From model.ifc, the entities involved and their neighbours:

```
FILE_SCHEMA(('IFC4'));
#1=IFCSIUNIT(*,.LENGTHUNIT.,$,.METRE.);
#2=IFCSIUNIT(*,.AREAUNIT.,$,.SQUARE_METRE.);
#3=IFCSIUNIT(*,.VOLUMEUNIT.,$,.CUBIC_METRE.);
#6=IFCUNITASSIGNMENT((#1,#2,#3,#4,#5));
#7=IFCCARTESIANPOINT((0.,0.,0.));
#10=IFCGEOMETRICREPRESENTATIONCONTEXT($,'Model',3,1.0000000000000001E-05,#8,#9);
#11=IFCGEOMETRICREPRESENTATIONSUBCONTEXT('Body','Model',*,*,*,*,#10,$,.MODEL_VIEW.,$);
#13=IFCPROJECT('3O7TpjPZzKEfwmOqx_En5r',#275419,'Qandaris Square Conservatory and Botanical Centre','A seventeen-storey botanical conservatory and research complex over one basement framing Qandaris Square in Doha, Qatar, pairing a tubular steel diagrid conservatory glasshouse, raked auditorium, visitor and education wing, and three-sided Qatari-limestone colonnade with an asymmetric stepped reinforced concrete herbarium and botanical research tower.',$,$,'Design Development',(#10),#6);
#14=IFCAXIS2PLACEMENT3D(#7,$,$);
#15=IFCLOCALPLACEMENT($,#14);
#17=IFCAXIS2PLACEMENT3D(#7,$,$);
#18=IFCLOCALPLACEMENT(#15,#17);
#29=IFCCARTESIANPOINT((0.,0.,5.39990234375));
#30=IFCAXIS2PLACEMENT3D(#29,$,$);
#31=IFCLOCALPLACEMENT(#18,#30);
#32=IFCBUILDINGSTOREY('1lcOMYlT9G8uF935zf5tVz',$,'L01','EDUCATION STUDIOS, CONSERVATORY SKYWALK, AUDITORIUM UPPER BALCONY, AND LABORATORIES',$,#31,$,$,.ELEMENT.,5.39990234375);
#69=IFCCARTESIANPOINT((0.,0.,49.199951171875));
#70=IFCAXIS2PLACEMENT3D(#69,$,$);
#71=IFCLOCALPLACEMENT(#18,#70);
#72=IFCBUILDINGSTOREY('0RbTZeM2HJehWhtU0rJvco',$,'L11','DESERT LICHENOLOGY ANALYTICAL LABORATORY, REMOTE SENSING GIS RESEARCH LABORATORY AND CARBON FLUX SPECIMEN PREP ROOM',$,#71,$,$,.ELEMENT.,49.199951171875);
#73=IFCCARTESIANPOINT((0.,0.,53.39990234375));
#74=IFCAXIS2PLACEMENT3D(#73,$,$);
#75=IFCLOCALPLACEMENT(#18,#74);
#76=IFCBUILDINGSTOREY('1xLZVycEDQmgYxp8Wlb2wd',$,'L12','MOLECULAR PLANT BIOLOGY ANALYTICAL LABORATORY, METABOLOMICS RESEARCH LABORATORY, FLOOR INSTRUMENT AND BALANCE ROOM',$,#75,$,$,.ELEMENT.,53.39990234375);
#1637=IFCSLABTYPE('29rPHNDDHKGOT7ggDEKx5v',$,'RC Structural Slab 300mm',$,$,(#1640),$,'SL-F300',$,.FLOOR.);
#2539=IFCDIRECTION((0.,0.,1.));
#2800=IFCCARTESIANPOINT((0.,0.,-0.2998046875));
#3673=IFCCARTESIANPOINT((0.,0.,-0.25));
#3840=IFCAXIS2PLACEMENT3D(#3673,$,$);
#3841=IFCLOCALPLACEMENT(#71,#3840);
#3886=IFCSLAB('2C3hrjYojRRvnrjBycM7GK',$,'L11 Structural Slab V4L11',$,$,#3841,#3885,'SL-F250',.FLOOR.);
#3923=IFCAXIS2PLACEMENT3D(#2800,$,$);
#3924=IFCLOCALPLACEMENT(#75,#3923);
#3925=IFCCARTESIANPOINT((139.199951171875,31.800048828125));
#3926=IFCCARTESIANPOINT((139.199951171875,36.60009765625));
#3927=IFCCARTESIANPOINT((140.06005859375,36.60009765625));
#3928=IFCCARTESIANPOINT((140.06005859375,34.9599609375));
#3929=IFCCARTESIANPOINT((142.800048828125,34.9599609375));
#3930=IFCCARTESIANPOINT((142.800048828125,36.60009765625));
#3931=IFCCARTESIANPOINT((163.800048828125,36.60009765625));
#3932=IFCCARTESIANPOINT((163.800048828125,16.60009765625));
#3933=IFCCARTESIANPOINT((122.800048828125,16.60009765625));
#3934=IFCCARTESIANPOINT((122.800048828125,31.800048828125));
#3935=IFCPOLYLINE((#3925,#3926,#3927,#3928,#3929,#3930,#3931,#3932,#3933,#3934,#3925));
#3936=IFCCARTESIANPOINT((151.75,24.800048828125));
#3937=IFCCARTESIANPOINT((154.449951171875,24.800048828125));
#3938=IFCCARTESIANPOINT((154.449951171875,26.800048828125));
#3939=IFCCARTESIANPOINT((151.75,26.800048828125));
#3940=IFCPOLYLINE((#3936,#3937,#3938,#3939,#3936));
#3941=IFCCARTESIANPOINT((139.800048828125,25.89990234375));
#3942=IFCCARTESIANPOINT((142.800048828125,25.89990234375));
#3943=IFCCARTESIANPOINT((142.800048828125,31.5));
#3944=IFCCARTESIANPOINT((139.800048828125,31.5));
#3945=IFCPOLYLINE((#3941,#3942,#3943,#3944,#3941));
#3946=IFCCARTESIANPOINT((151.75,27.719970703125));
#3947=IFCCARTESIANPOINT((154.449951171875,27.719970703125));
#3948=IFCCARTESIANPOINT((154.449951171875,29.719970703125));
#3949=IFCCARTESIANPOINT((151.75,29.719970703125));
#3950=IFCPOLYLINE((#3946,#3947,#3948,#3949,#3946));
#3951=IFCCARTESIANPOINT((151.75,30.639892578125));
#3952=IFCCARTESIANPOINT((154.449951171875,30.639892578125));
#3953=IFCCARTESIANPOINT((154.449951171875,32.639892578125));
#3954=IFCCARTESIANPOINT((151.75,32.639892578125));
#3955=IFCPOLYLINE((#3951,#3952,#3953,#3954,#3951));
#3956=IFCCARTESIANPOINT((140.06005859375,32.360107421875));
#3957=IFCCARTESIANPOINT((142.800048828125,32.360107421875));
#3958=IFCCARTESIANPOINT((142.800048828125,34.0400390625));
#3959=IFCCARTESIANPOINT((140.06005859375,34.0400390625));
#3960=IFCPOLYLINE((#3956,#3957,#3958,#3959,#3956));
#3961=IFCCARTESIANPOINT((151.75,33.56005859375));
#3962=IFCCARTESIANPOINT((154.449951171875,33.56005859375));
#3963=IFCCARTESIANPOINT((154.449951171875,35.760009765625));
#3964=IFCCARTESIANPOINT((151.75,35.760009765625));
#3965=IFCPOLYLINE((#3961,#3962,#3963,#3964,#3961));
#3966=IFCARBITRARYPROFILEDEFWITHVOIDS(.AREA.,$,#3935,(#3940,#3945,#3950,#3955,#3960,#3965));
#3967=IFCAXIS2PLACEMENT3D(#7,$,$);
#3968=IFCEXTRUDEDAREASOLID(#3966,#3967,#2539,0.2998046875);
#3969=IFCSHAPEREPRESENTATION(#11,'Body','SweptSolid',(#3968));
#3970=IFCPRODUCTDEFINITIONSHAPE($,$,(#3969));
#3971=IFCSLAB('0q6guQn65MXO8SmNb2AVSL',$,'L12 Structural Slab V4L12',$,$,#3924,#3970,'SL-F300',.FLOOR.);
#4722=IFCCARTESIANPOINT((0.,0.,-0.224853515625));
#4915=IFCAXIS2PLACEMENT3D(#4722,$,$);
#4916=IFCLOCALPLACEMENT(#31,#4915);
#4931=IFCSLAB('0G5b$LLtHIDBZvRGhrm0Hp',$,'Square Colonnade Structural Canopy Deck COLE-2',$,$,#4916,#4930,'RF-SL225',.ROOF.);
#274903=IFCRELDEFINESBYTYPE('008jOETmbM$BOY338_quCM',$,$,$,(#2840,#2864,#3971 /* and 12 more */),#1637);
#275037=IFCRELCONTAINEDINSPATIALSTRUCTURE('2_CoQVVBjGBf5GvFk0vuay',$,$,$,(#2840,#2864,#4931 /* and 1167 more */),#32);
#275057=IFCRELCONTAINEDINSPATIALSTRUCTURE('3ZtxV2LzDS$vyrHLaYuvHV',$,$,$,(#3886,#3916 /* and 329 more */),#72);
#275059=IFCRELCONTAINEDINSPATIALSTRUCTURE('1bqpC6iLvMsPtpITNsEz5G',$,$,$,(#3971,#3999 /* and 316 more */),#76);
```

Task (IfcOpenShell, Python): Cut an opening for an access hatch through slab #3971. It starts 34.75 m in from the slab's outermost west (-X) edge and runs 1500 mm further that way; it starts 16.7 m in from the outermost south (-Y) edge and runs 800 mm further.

```python
import numpy as np
import ifcopenshell
import ifcopenshell.api.feature
import ifcopenshell.api.geometry
import ifcopenshell.api.root
import ifcopenshell.geom
import ifcopenshell.util.placement
import ifcopenshell.util.representation
import ifcopenshell.util.shape
import ifcopenshell.util.unit

model = ifcopenshell.open("model.ifc")
unit_scale = ifcopenshell.util.unit.calculate_unit_scale(model)
settings = ifcopenshell.geom.settings()


def volume(element):
    """Net volume in cubic metres, openings subtracted."""
    shape = ifcopenshell.geom.create_shape(settings, element)
    return ifcopenshell.util.shape.get_volume(shape.geometry)


slab = model.by_guid("0q6guQn65MXO8SmNb2AVSL")
before = volume(slab)

# Extent in the slab's own axes, in metres. The edges named are its -X and -Y sides.
slab_shape = ifcopenshell.geom.create_shape(settings, slab)
vertices = ifcopenshell.util.shape.get_vertices(slab_shape.geometry)
x_min, y_min, bottom = vertices.min(axis=0)
top = vertices[:, 2].max()

opening = ifcopenshell.api.root.create_entity(model, ifc_class="IfcOpeningElement", name="Access hatch opening", predefined_type="OPENING")
context = ifcopenshell.util.representation.get_context(model, "Model", "Body", "MODEL_VIEW")
width, depth = 1.5, 0.8
outline = [(0.0, 0.0), (width, 0.0), (width, depth), (0.0, depth), (0.0, 0.0)]
# Overshoot both faces by 50 mm so the cut is clean.
shape = ifcopenshell.api.geometry.add_slab_representation(
    model, context=context, depth=top - bottom + 0.1, polyline=outline
)
ifcopenshell.api.geometry.assign_representation(model, product=opening, representation=shape)

matrix = ifcopenshell.util.placement.get_local_placement(slab.ObjectPlacement)
matrix[:, 3] = matrix @ np.append(np.array([x_min + 34.75, y_min + 16.7, bottom - 0.05]) / unit_scale, 1.0)
ifcopenshell.api.geometry.edit_object_placement(model, product=opening, matrix=matrix, is_si=False)
ifcopenshell.api.feature.add_feature(model, feature=opening, element=slab)

after = volume(slab)

print(f"slab volume {before:.3f} -> {after:.3f} m3")

model.write("model_updated.ifc")
```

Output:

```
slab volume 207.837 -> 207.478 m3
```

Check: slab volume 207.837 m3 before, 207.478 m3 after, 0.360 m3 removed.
